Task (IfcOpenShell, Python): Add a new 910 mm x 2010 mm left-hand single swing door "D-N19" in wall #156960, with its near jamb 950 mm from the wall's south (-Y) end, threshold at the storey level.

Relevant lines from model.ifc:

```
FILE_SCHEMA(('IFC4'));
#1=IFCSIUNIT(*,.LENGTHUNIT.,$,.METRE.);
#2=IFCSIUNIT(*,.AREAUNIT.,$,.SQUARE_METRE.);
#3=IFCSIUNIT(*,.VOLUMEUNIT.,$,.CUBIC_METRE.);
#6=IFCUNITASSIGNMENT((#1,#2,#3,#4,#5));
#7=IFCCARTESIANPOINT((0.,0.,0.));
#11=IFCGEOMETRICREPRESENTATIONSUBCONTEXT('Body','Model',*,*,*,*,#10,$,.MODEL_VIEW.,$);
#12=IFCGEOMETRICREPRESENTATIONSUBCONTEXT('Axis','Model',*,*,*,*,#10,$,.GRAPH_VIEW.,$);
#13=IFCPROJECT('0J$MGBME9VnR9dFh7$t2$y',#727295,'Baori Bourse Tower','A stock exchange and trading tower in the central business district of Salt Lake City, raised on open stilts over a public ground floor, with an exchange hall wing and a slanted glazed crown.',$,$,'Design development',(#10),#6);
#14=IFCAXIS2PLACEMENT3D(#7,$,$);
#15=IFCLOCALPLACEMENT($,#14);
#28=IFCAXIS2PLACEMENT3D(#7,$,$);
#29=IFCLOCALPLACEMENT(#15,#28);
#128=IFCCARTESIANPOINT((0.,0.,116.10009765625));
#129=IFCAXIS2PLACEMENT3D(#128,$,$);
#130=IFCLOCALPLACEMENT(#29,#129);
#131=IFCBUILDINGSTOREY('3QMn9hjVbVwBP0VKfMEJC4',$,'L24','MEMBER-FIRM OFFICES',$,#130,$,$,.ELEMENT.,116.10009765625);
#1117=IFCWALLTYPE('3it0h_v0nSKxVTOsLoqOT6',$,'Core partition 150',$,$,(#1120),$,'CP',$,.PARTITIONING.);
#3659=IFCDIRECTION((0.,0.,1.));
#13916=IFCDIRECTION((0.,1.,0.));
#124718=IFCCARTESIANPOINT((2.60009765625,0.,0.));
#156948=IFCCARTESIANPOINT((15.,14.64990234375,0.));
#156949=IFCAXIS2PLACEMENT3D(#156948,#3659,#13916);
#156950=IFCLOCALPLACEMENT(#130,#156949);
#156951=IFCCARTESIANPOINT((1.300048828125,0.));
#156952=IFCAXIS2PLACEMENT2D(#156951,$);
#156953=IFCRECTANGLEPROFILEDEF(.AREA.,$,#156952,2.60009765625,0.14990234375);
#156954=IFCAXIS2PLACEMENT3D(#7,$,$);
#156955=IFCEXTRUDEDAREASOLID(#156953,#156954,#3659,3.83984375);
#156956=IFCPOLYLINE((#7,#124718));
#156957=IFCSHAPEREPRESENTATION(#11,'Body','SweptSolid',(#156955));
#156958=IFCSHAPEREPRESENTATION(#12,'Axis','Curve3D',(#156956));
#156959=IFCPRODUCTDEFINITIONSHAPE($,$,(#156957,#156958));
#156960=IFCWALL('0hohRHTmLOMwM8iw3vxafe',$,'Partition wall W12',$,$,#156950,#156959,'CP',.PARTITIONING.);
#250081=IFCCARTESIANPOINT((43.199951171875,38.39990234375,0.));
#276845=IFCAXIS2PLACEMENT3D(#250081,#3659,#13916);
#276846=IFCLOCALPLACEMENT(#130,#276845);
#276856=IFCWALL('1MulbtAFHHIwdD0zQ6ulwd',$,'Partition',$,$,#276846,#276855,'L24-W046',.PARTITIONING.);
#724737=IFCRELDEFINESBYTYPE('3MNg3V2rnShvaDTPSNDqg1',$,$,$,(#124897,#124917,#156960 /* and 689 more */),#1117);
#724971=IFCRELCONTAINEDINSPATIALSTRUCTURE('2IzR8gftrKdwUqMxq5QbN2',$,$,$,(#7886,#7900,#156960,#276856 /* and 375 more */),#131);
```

```python
import numpy as np
import ifcopenshell
import ifcopenshell.api.feature
import ifcopenshell.api.geometry
import ifcopenshell.api.root
import ifcopenshell.api.spatial
import ifcopenshell.geom
import ifcopenshell.util.element
import ifcopenshell.util.placement
import ifcopenshell.util.representation
import ifcopenshell.util.shape
import ifcopenshell.util.unit

model = ifcopenshell.open("model.ifc")
unit_scale = ifcopenshell.util.unit.calculate_unit_scale(model)
settings = ifcopenshell.geom.settings()


def volume(element):
    """Net volume in cubic metres, openings subtracted."""
    shape = ifcopenshell.geom.create_shape(settings, element)
    return ifcopenshell.util.shape.get_volume(shape.geometry)


wall = model.by_id(156960)
storey = ifcopenshell.util.element.get_container(wall, ifc_class="IfcBuildingStorey")
context = ifcopenshell.util.representation.get_context(model, "Model", "Body", "MODEL_VIEW")
before = volume(wall)

width, height, from_end, sill = 0.91, 2.01, 0.95, 0.0  # metres

# The wall runs along its own X axis, and the end named is its -X end.
wall_shape = ifcopenshell.geom.create_shape(settings, wall)
x, y, z = ifcopenshell.util.shape.get_vertices(wall_shape.geometry).T
start = x.min() + from_end
face, thickness = float(y.min()), float(y.max() - y.min())
wall_matrix = ifcopenshell.util.placement.get_local_placement(wall.ObjectPlacement)
level = ifcopenshell.util.placement.get_local_placement(storey.ObjectPlacement)[2, 3]


def in_wall(x, y):
    """Placement at x, y metres in the wall's axes, at sill height."""
    matrix = wall_matrix.copy()
    matrix[:, 3] = wall_matrix @ np.array([x / unit_scale, y / unit_scale, 0.0, 1.0])
    matrix[2, 3] = level + sill / unit_scale
    return matrix


# Opening: a box that overshoots both wall faces by 50 mm.
opening = ifcopenshell.api.root.create_entity(model, ifc_class="IfcOpeningElement", predefined_type="OPENING")
box = ifcopenshell.api.geometry.add_wall_representation(
    model, context=context, length=width, height=height, thickness=thickness + 0.1
)
ifcopenshell.api.geometry.assign_representation(model, product=opening, representation=box)
ifcopenshell.api.geometry.edit_object_placement(model, product=opening, matrix=in_wall(start, face - 0.05), is_si=False)
ifcopenshell.api.feature.add_feature(model, feature=opening, element=wall)

door = ifcopenshell.api.root.create_entity(model, ifc_class="IfcDoor", name="D-N19", predefined_type="DOOR")
door.OverallWidth, door.OverallHeight = width / unit_scale, height / unit_scale
door.OperationType = "SINGLE_SWING_LEFT"
body = ifcopenshell.api.geometry.add_door_representation(
    model,
    context=context,
    overall_width=door.OverallWidth,
    overall_height=door.OverallHeight,
    operation_type="SINGLE_SWING_LEFT",
    lining_properties={"LiningDepth": thickness / unit_scale, "ThresholdDepth": thickness / unit_scale},
)
ifcopenshell.api.geometry.assign_representation(model, product=door, representation=body)
ifcopenshell.api.spatial.assign_container(model, products=[door], relating_structure=storey)
ifcopenshell.api.feature.add_filling(model, opening=opening, element=door)

# The lining spans the wall, so the door starts at the wall face.
ifcopenshell.api.geometry.edit_object_placement(model, product=door, matrix=in_wall(start, face), is_si=False)

after = volume(wall)

print(f"wall volume {before:.3f} -> {after:.3f} m3")

model.write("model_v2.ifc")
```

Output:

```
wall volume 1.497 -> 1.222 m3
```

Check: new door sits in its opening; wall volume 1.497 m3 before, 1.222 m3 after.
